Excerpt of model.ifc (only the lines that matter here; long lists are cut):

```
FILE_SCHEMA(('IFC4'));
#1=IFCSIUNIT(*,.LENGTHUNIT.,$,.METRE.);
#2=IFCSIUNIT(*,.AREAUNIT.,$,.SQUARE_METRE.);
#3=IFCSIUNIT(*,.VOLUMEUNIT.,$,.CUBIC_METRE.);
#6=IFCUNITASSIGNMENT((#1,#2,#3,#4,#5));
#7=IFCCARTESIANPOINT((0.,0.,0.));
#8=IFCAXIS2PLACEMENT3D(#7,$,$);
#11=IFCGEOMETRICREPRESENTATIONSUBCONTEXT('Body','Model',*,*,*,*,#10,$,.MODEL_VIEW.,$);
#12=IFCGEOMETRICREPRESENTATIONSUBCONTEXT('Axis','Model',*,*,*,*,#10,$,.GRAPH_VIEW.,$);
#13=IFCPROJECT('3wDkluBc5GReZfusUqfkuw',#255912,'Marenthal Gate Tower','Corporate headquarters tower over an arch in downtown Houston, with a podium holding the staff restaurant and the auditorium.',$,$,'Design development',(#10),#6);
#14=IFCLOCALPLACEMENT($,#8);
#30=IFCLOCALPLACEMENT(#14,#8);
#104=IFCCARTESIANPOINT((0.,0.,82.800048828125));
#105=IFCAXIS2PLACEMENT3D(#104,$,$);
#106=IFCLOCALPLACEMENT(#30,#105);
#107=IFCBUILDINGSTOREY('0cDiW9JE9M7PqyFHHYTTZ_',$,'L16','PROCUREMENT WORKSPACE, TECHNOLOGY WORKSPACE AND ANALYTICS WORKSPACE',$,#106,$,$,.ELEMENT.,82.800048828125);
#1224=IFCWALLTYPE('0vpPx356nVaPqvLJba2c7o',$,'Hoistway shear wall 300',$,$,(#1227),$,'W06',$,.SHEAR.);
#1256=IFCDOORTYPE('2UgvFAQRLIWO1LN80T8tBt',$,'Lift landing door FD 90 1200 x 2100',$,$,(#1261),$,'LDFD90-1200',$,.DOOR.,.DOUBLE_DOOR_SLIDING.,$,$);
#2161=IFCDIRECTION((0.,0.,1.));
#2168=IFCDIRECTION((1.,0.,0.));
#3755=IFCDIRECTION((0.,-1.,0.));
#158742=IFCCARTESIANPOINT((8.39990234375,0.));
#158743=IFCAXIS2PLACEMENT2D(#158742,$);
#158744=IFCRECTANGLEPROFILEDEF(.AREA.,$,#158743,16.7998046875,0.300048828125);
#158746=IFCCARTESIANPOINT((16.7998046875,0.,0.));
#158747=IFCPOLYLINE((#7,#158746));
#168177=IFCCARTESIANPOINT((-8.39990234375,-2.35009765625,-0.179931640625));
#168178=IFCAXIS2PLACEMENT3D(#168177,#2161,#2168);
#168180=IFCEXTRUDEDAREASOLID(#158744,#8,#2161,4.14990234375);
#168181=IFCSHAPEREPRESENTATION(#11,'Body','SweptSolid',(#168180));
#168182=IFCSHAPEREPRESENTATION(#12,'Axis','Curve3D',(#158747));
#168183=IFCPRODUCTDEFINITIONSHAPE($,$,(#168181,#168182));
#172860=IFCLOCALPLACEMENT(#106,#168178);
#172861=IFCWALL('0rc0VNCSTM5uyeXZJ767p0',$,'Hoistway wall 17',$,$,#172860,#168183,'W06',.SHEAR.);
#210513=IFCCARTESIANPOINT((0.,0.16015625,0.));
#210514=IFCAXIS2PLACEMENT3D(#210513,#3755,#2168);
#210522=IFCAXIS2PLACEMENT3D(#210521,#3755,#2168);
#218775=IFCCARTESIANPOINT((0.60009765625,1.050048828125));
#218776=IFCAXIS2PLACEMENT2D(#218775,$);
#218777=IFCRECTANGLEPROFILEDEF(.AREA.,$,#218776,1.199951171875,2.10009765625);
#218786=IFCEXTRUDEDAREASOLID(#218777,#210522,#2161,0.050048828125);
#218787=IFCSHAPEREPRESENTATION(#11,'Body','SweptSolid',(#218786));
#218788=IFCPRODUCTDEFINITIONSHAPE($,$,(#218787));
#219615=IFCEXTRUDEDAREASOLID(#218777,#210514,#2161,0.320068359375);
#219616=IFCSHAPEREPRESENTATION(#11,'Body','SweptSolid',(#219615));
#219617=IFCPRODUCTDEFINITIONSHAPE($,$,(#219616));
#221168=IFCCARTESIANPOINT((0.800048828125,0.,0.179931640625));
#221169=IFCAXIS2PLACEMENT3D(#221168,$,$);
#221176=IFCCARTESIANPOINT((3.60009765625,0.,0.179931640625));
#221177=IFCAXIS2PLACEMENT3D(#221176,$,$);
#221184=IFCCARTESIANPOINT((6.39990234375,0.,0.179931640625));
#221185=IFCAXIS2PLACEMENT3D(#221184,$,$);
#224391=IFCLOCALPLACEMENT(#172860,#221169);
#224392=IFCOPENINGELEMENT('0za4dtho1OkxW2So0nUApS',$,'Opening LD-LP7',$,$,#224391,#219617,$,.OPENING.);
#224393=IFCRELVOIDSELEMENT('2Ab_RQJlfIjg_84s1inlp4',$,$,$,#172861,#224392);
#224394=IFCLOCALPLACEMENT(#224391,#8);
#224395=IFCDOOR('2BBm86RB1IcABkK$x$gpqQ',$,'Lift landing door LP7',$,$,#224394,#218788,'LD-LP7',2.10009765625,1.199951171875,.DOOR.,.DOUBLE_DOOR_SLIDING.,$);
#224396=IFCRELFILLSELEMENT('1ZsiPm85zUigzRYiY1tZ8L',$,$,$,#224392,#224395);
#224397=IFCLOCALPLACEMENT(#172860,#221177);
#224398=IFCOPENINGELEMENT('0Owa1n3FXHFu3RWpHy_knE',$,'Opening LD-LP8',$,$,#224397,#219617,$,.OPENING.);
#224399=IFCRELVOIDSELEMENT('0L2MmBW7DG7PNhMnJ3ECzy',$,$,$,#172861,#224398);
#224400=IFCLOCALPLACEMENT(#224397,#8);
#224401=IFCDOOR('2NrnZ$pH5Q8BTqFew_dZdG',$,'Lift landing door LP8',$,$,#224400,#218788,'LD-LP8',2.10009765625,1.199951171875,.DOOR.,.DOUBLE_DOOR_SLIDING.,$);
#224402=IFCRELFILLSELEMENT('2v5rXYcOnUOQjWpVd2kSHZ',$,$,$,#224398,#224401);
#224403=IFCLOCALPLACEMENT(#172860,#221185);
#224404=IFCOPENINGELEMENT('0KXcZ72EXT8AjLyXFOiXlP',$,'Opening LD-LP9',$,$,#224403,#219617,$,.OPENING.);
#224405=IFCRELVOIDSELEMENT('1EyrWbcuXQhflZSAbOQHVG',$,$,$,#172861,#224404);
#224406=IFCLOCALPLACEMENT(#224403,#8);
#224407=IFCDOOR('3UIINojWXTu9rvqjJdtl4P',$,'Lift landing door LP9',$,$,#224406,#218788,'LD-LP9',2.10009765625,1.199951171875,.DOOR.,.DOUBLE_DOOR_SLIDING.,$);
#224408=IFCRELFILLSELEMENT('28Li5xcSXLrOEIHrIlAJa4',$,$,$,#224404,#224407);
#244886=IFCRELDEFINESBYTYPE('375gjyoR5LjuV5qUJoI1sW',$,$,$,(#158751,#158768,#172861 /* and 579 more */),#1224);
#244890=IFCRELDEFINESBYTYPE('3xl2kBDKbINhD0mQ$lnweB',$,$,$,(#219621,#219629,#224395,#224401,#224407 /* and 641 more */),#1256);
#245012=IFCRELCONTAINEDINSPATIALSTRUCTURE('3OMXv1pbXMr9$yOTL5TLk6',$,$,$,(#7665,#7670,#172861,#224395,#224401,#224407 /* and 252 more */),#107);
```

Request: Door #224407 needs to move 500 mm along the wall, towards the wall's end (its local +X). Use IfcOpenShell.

```python
import ifcopenshell
import ifcopenshell.api.geometry
import ifcopenshell.util.placement

model = ifcopenshell.open("model.ifc")

door = model.by_guid("3UIINojWXTu9rvqjJdtl4P")
opening = door.FillsVoids[0].RelatingOpeningElement
wall = opening.VoidsElements[0].RelatingBuildingElement

wall_matrix = ifcopenshell.util.placement.get_local_placement(wall.ObjectPlacement)
shift = wall_matrix[:3, 0] * 0.5
before = ifcopenshell.util.placement.get_local_placement(door.ObjectPlacement)[:3, 3].copy()

# The door is placed relative to its opening, so it follows when the opening moves.
matrix = ifcopenshell.util.placement.get_local_placement(opening.ObjectPlacement)
matrix[:3, 3] += shift
ifcopenshell.api.geometry.edit_object_placement(
    model, product=opening, matrix=matrix, is_si=False, should_transform_children=True
)

after = ifcopenshell.util.placement.get_local_placement(door.ObjectPlacement)[:3, 3]
print("door moved by", (after - before).round(3) + 0.0)

model.write("model_v2.ifc")
```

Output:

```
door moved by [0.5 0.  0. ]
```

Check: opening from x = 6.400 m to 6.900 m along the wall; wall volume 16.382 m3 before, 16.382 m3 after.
